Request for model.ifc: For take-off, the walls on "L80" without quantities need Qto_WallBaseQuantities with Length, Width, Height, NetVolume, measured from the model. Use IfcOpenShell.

First a look at what the model holds.

```python
import ifcopenshell
import ifcopenshell.util.element
import ifcopenshell.util.unit

model = ifcopenshell.open("model.ifc")
print(model.schema)
for unit_type in ("LENGTHUNIT", "AREAUNIT", "VOLUMEUNIT"):
    print(unit_type, ifcopenshell.util.unit.calculate_unit_scale(model, unit_type))
storey = next(s for s in model.by_type("IfcBuildingStorey") if s.Name == "L80")
walls = [e for e in ifcopenshell.util.element.get_decomposition(storey) if e.is_a("IfcWall")]
for e in sorted(walls, key=lambda e: e.id()):
    print(e.id(), e.is_a(), e.Name, list(ifcopenshell.util.element.get_psets(e, qtos_only=True)), sep=" | ")
```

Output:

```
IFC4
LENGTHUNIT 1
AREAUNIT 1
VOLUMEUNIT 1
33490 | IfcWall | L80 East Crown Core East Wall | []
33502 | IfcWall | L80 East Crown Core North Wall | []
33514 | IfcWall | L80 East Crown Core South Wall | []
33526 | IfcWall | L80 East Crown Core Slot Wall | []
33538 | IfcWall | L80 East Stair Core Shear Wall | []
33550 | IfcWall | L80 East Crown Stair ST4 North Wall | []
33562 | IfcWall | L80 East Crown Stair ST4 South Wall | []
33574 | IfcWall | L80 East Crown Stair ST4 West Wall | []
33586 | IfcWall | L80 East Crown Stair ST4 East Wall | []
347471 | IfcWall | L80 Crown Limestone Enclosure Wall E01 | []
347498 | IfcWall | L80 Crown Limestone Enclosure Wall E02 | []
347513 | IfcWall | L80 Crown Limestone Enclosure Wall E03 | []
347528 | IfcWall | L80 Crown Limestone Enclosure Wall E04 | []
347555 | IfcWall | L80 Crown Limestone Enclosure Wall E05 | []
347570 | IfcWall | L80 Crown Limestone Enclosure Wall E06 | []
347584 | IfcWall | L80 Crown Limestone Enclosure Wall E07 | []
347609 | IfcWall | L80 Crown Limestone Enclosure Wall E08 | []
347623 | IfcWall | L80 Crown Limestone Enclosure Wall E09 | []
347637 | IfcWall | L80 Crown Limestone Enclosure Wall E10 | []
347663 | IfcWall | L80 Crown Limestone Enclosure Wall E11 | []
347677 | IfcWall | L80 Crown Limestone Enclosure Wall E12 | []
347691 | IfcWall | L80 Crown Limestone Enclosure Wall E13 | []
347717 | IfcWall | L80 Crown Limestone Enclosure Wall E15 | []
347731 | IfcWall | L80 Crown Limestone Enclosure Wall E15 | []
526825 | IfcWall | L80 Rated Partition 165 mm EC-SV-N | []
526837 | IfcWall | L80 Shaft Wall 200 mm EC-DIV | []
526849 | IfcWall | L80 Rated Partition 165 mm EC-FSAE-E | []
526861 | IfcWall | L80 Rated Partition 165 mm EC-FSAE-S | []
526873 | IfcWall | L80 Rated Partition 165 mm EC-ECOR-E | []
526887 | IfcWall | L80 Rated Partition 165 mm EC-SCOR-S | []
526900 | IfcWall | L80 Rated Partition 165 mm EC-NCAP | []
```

```python
import ifcopenshell
import ifcopenshell.api.pset
import ifcopenshell.geom
import ifcopenshell.util.element
import ifcopenshell.util.shape
import ifcopenshell.util.unit

model = ifcopenshell.open("model.ifc")
unit_scale = ifcopenshell.util.unit.calculate_unit_scale(model)
volume_scale = ifcopenshell.util.unit.calculate_unit_scale(model, "VOLUMEUNIT")
settings = ifcopenshell.geom.settings()

storey = next(s for s in model.by_type("IfcBuildingStorey") if s.Name == "L80")
walls = [e for e in ifcopenshell.util.element.get_decomposition(storey) if e.is_a("IfcWall")]

for e in sorted(walls, key=lambda e: e.id()):
    if ifcopenshell.util.element.get_psets(e, qtos_only=True, should_inherit=False):
        continue
    # Geometry comes back in metres, in the element's own axes.
    shape = ifcopenshell.geom.create_shape(settings, e)
    values = {
        "Length": ifcopenshell.util.shape.get_x(shape.geometry) / unit_scale,
        "Width": ifcopenshell.util.shape.get_y(shape.geometry) / unit_scale,
        "Height": ifcopenshell.util.shape.get_z(shape.geometry) / unit_scale,
        "NetVolume": ifcopenshell.util.shape.get_volume(shape.geometry) / volume_scale,
    }
    qto = ifcopenshell.api.pset.add_qto(model, product=e, name="Qto_WallBaseQuantities")
    ifcopenshell.api.pset.edit_qto(model, qto=qto, properties=values)
    print(e.id(), {k: round(v, 3) for k, v in values.items()})

model.write("model_rev.ifc")
```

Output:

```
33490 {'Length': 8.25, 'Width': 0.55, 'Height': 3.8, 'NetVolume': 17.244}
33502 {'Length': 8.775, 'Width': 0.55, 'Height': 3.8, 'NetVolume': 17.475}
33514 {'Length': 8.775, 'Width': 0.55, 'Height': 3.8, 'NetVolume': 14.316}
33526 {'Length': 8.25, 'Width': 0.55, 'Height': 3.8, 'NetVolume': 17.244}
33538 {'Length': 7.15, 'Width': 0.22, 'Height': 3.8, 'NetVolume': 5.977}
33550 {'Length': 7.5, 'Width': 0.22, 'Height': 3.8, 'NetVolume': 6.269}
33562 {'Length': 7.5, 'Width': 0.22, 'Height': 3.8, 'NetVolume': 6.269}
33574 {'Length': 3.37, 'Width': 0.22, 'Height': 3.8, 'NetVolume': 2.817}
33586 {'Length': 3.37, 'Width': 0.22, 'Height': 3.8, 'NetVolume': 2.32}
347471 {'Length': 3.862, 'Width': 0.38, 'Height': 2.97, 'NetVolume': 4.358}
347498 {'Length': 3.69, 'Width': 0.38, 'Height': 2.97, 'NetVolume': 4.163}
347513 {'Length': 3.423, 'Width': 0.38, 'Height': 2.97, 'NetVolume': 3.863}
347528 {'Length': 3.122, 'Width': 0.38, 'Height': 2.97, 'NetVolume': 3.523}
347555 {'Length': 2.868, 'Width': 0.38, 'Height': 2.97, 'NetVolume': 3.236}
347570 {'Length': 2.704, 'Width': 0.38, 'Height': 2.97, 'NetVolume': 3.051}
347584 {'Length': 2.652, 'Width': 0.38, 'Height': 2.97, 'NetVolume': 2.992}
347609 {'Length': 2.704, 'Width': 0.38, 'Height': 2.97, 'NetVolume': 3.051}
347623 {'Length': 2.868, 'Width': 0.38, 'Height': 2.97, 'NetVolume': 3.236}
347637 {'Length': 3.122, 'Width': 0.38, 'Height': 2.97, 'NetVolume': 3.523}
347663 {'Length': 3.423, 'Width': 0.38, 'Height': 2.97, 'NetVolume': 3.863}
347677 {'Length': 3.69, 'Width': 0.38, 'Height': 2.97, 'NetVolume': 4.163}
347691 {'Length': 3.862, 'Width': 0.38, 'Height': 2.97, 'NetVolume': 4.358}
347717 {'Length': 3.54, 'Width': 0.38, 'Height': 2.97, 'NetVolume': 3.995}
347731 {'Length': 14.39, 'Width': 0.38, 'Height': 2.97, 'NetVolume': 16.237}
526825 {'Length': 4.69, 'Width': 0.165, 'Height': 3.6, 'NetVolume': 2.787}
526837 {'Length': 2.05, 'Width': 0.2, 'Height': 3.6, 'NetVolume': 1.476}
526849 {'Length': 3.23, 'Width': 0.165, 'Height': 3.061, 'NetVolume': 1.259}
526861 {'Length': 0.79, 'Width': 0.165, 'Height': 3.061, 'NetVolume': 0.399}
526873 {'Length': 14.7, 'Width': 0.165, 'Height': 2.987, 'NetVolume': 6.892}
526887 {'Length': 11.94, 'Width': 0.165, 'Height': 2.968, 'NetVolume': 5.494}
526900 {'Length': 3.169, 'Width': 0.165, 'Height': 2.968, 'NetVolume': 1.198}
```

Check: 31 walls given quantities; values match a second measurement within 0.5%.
